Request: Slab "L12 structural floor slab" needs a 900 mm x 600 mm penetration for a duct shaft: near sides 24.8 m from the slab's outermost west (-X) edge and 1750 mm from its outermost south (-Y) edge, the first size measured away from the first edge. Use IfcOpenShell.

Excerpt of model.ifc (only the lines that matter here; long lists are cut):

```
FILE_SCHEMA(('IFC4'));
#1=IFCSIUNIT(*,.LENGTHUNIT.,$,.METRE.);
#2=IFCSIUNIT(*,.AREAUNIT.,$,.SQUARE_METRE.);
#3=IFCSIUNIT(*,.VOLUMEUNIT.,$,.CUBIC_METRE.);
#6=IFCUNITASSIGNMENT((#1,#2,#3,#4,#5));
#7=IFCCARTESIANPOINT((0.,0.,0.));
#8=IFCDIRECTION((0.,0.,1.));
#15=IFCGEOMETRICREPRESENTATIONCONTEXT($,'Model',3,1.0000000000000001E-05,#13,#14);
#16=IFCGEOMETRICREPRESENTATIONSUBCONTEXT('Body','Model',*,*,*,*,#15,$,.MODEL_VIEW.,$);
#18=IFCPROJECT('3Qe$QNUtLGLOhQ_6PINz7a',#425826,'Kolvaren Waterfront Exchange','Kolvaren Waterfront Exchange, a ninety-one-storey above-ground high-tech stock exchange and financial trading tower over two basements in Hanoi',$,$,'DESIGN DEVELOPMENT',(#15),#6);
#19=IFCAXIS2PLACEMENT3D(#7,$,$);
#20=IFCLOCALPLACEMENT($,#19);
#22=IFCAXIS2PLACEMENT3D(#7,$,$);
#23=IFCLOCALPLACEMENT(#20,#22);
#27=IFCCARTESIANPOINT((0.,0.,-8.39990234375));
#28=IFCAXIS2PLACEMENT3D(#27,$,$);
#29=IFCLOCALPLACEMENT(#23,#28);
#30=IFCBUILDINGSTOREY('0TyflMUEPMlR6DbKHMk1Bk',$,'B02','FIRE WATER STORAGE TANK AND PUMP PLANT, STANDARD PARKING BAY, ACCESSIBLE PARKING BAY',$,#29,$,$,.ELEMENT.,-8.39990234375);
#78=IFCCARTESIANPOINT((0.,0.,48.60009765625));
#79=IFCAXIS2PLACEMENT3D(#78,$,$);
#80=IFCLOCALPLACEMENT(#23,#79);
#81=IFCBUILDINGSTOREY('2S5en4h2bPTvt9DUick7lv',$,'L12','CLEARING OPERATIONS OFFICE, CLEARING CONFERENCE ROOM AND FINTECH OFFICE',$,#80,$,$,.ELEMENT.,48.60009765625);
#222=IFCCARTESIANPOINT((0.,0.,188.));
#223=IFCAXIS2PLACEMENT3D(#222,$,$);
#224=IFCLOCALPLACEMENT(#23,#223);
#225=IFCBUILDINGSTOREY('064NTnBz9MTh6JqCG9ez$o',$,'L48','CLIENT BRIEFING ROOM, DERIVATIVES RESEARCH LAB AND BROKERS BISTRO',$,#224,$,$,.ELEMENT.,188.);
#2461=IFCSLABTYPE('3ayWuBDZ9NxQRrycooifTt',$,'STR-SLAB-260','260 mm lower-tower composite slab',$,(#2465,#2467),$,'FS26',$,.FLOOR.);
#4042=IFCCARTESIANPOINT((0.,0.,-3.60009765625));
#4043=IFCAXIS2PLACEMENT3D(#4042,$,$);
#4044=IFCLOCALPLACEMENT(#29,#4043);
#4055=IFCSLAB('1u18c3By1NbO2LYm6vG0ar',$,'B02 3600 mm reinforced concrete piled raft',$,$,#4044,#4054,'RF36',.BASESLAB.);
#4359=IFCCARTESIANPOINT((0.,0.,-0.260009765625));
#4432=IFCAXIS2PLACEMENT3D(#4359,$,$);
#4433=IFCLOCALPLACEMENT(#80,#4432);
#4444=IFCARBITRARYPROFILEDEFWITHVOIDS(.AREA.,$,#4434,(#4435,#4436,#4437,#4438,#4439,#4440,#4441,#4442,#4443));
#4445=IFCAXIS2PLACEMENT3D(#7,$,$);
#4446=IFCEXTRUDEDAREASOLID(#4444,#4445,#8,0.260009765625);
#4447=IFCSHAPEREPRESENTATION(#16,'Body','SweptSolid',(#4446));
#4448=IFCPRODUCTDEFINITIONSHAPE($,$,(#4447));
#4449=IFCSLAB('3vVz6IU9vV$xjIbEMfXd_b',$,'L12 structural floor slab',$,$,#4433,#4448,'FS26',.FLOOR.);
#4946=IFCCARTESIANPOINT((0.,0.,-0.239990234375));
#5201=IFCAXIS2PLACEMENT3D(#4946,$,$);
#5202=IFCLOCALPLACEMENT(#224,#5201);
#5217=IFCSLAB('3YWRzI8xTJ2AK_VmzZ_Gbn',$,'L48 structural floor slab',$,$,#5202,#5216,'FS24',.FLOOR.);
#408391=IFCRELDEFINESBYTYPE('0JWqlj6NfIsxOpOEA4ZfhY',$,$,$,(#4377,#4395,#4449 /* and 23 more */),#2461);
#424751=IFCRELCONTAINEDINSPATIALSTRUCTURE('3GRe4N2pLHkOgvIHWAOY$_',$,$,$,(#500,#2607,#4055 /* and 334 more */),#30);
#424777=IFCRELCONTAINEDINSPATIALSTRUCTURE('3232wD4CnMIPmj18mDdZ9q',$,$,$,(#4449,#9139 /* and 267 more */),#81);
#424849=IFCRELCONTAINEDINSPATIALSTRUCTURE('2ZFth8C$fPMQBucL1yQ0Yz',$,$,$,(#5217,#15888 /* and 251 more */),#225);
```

```python
import numpy as np
import ifcopenshell
import ifcopenshell.api.feature
import ifcopenshell.api.geometry
import ifcopenshell.api.root
import ifcopenshell.geom
import ifcopenshell.util.placement
import ifcopenshell.util.representation
import ifcopenshell.util.shape
import ifcopenshell.util.unit

model = ifcopenshell.open("model.ifc")
unit_scale = ifcopenshell.util.unit.calculate_unit_scale(model)
settings = ifcopenshell.geom.settings()


def volume(element):
    """Net volume in cubic metres, openings subtracted."""
    shape = ifcopenshell.geom.create_shape(settings, element)
    return ifcopenshell.util.shape.get_volume(shape.geometry)


slab = model.by_guid("3vVz6IU9vV$xjIbEMfXd_b")
before = volume(slab)

# Extent in the slab's own axes, in metres. The edges named are its -X and -Y sides.
slab_shape = ifcopenshell.geom.create_shape(settings, slab)
vertices = ifcopenshell.util.shape.get_vertices(slab_shape.geometry)
x_min, y_min, bottom = vertices.min(axis=0)
top = vertices[:, 2].max()

opening = ifcopenshell.api.root.create_entity(model, ifc_class="IfcOpeningElement", name="Duct shaft opening", predefined_type="OPENING")
context = ifcopenshell.util.representation.get_context(model, "Model", "Body", "MODEL_VIEW")
width, depth = 0.9, 0.6
outline = [(0.0, 0.0), (width, 0.0), (width, depth), (0.0, depth), (0.0, 0.0)]
# Overshoot both faces by 50 mm so the cut is clean.
shape = ifcopenshell.api.geometry.add_slab_representation(
    model, context=context, depth=top - bottom + 0.1, polyline=outline
)
ifcopenshell.api.geometry.assign_representation(model, product=opening, representation=shape)

matrix = ifcopenshell.util.placement.get_local_placement(slab.ObjectPlacement)
matrix[:, 3] = matrix @ np.append(np.array([x_min + 24.8, y_min + 1.75, bottom - 0.05]) / unit_scale, 1.0)
ifcopenshell.api.geometry.edit_object_placement(model, product=opening, matrix=matrix, is_si=False)
ifcopenshell.api.feature.add_feature(model, feature=opening, element=slab)

after = volume(slab)

print(f"slab volume {before:.3f} -> {after:.3f} m3")

model.write("model_v2.ifc")
```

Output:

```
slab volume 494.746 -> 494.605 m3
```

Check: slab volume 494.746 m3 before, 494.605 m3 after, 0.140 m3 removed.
